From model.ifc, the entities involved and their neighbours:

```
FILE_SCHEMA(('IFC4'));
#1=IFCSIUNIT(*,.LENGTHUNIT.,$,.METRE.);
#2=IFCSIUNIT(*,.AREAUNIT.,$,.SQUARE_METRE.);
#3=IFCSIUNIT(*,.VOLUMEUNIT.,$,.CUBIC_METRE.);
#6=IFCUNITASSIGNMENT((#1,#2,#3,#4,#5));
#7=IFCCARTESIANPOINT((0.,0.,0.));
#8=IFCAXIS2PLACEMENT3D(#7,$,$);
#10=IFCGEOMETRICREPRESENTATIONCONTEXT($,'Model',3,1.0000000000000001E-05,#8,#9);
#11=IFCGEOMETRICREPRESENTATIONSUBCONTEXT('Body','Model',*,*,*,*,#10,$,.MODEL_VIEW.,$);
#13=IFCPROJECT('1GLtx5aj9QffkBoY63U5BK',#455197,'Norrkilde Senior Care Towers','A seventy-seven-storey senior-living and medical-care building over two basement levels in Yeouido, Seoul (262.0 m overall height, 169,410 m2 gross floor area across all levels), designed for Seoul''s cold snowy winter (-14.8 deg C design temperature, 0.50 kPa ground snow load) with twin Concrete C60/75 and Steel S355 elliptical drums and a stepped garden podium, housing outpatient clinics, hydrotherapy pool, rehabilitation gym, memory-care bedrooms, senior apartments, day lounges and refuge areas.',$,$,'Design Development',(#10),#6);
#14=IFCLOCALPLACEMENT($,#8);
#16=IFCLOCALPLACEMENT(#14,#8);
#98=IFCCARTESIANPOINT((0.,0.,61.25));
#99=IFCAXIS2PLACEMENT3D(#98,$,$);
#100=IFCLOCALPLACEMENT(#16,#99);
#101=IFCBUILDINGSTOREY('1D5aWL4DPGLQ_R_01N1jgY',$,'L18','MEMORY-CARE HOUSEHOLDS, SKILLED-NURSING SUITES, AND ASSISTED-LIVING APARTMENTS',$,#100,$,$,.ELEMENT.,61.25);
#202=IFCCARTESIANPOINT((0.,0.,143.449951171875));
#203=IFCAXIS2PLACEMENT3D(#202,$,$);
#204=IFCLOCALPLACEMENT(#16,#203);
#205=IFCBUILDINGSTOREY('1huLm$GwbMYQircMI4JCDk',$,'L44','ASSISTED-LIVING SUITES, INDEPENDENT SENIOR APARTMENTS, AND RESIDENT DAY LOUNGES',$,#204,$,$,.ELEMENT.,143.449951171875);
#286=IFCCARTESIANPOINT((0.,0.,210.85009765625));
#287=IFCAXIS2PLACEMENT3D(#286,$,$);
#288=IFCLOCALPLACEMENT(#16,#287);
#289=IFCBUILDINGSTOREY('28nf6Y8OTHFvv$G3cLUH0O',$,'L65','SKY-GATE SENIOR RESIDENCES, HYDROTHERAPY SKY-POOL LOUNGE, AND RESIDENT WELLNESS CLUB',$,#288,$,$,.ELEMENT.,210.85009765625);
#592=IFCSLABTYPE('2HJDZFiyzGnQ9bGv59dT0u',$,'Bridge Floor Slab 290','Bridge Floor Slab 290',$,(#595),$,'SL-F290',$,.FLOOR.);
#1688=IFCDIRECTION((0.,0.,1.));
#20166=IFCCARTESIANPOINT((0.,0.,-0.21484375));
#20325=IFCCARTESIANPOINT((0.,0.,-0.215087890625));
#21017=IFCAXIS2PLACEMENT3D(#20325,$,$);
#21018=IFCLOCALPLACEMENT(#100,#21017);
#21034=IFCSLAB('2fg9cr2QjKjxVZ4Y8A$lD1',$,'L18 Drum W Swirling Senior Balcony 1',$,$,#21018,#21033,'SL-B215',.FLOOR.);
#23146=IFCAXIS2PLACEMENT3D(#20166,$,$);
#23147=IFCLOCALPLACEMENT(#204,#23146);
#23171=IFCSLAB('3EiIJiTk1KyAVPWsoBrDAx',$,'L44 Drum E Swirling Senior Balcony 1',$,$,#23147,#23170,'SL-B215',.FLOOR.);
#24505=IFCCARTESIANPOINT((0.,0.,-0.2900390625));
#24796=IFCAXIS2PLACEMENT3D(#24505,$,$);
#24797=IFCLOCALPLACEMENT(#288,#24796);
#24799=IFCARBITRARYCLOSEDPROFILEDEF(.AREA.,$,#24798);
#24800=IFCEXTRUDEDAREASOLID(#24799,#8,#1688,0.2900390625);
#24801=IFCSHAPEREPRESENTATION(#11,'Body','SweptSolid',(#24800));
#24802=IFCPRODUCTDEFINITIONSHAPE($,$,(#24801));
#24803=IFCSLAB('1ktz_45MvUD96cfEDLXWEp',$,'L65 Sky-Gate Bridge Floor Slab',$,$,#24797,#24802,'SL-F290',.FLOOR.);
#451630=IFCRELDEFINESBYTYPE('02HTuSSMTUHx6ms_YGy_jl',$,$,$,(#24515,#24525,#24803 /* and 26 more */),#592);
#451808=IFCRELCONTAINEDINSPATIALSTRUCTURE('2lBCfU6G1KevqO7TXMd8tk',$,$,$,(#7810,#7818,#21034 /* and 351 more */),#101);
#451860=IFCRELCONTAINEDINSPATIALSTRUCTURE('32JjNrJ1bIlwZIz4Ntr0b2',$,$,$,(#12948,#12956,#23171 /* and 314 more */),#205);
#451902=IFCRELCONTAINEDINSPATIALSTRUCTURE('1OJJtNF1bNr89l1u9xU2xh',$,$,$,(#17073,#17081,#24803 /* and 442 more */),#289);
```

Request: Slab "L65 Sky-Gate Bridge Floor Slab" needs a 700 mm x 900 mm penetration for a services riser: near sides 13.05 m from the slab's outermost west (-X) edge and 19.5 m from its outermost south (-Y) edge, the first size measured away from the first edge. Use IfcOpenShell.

```python
import numpy as np
import ifcopenshell
import ifcopenshell.api.feature
import ifcopenshell.api.geometry
import ifcopenshell.api.root
import ifcopenshell.geom
import ifcopenshell.util.placement
import ifcopenshell.util.representation
import ifcopenshell.util.shape
import ifcopenshell.util.unit

model = ifcopenshell.open("model.ifc")
unit_scale = ifcopenshell.util.unit.calculate_unit_scale(model)
settings = ifcopenshell.geom.settings()


def volume(element):
    """Net volume in cubic metres, openings subtracted."""
    shape = ifcopenshell.geom.create_shape(settings, element)
    return ifcopenshell.util.shape.get_volume(shape.geometry)


slab = model.by_guid("1ktz_45MvUD96cfEDLXWEp")
before = volume(slab)

# Extent in the slab's own axes, in metres. The edges named are its -X and -Y sides.
slab_shape = ifcopenshell.geom.create_shape(settings, slab)
vertices = ifcopenshell.util.shape.get_vertices(slab_shape.geometry)
x_min, y_min, bottom = vertices.min(axis=0)
top = vertices[:, 2].max()

opening = ifcopenshell.api.root.create_entity(model, ifc_class="IfcOpeningElement", name="Services riser opening", predefined_type="OPENING")
context = ifcopenshell.util.representation.get_context(model, "Model", "Body", "MODEL_VIEW")
width, depth = 0.7, 0.9
outline = [(0.0, 0.0), (width, 0.0), (width, depth), (0.0, depth), (0.0, 0.0)]
# Overshoot both faces by 50 mm so the cut is clean.
shape = ifcopenshell.api.geometry.add_slab_representation(
    model, context=context, depth=top - bottom + 0.1, polyline=outline
)
ifcopenshell.api.geometry.assign_representation(model, product=opening, representation=shape)

matrix = ifcopenshell.util.placement.get_local_placement(slab.ObjectPlacement)
matrix[:, 3] = matrix @ np.append(np.array([x_min + 13.05, y_min + 19.5, bottom - 0.05]) / unit_scale, 1.0)
ifcopenshell.api.geometry.edit_object_placement(model, product=opening, matrix=matrix, is_si=False)
ifcopenshell.api.feature.add_feature(model, feature=opening, element=slab)

after = volume(slab)

print(f"slab volume {before:.3f} -> {after:.3f} m3")

model.write("model_updated.ifc")
```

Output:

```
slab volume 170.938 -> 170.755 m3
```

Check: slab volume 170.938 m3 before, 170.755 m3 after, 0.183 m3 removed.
